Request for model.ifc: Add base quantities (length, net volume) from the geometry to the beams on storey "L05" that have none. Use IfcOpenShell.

First a look at what the model holds.

```python
import ifcopenshell
import ifcopenshell.util.element
import ifcopenshell.util.unit

model = ifcopenshell.open("model.ifc")
print(model.schema)
for unit_type in ("LENGTHUNIT", "AREAUNIT", "VOLUMEUNIT"):
    print(unit_type, ifcopenshell.util.unit.calculate_unit_scale(model, unit_type))
storey = next(s for s in model.by_type("IfcBuildingStorey") if s.Name == "L05")
beams = [e for e in ifcopenshell.util.element.get_decomposition(storey) if e.is_a("IfcBeam")]
for e in sorted(beams, key=lambda e: e.id()):
    print(e.id(), e.is_a(), e.Name, list(ifcopenshell.util.element.get_psets(e, qtos_only=True)), sep=" | ")
```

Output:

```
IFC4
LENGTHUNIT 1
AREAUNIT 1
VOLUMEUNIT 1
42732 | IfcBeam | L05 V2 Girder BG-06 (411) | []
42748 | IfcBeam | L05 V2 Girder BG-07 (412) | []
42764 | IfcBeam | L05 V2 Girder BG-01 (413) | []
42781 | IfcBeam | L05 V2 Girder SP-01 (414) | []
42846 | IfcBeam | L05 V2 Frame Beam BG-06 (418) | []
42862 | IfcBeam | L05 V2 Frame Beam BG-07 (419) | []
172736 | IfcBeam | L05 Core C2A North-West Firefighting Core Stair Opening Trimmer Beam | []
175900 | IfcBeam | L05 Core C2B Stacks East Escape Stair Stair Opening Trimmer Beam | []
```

```python
import ifcopenshell
import ifcopenshell.api.pset
import ifcopenshell.geom
import ifcopenshell.util.element
import ifcopenshell.util.shape
import ifcopenshell.util.unit

model = ifcopenshell.open("model.ifc")
unit_scale = ifcopenshell.util.unit.calculate_unit_scale(model)
volume_scale = ifcopenshell.util.unit.calculate_unit_scale(model, "VOLUMEUNIT")
settings = ifcopenshell.geom.settings()

storey = next(s for s in model.by_type("IfcBuildingStorey") if s.Name == "L05")
beams = [e for e in ifcopenshell.util.element.get_decomposition(storey) if e.is_a("IfcBeam")]

for e in sorted(beams, key=lambda e: e.id()):
    if ifcopenshell.util.element.get_psets(e, qtos_only=True, should_inherit=False):
        continue
    # Geometry comes back in metres, in the element's own axes.
    shape = ifcopenshell.geom.create_shape(settings, e)
    values = {
        "Length": ifcopenshell.util.shape.get_max_xyz(shape.geometry) / unit_scale,
        "NetVolume": ifcopenshell.util.shape.get_volume(shape.geometry) / volume_scale,
    }
    qto = ifcopenshell.api.pset.add_qto(model, product=e, name="Qto_BeamBaseQuantities")
    ifcopenshell.api.pset.edit_qto(model, qto=qto, properties=values)
    print(e.id(), {k: round(v, 3) for k, v in values.items()})

model.write("model_rev.ifc")
```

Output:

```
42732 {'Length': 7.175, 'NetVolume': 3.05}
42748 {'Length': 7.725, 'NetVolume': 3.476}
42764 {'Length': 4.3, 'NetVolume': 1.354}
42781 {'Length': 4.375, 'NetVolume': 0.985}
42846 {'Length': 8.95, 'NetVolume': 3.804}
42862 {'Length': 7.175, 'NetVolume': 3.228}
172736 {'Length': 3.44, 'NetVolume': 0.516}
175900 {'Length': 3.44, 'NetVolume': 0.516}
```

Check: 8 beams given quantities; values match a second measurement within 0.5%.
